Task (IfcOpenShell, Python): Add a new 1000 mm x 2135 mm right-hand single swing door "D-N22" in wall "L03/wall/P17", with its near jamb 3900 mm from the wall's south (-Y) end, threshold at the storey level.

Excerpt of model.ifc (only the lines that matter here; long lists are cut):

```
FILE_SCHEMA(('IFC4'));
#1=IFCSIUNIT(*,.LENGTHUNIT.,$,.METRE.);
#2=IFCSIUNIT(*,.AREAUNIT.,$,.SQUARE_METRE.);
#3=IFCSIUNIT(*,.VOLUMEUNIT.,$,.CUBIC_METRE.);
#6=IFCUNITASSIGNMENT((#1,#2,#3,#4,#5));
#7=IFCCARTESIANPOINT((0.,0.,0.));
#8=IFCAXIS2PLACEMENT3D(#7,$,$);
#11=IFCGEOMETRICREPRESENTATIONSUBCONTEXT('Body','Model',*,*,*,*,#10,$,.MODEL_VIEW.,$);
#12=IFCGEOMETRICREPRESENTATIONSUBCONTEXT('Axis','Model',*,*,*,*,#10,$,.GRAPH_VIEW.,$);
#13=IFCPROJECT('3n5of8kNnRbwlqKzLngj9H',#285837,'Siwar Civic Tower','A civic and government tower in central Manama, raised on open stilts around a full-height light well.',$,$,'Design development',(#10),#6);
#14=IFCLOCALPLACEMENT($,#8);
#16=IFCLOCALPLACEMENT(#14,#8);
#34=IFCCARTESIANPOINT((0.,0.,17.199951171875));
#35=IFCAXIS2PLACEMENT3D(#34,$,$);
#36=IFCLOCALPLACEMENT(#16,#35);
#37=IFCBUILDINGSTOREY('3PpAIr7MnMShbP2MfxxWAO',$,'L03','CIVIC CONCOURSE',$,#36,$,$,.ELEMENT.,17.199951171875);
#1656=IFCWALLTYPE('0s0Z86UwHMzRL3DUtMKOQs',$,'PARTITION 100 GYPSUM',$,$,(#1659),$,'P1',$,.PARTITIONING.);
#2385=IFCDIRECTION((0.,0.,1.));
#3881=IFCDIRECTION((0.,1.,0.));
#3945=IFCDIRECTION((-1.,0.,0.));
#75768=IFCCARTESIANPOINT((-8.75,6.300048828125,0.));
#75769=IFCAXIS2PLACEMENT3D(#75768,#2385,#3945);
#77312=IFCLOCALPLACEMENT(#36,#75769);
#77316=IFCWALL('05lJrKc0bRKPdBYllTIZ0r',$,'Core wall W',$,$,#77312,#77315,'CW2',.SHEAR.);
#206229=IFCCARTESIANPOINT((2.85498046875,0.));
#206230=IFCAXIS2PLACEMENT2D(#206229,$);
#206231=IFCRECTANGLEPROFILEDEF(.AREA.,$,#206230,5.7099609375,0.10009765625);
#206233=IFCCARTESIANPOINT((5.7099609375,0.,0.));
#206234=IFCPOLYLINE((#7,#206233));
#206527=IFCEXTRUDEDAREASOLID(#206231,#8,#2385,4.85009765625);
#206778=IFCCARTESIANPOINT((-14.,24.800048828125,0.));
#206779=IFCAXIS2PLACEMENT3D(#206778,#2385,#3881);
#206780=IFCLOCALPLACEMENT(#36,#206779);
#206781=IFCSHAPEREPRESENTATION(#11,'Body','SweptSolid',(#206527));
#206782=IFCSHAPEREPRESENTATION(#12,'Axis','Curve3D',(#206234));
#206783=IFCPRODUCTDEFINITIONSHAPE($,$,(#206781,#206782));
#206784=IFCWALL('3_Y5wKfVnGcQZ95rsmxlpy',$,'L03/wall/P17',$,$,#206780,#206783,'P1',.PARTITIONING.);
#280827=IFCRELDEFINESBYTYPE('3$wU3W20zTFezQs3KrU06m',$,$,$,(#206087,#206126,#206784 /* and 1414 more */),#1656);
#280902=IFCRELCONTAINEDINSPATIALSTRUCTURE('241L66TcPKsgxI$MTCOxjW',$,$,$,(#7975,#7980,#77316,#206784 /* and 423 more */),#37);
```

```python
import numpy as np
import ifcopenshell
import ifcopenshell.api.feature
import ifcopenshell.api.geometry
import ifcopenshell.api.root
import ifcopenshell.api.spatial
import ifcopenshell.geom
import ifcopenshell.util.element
import ifcopenshell.util.placement
import ifcopenshell.util.representation
import ifcopenshell.util.shape
import ifcopenshell.util.unit

model = ifcopenshell.open("model.ifc")
unit_scale = ifcopenshell.util.unit.calculate_unit_scale(model)
settings = ifcopenshell.geom.settings()


def volume(element):
    """Net volume in cubic metres, openings subtracted."""
    shape = ifcopenshell.geom.create_shape(settings, element)
    return ifcopenshell.util.shape.get_volume(shape.geometry)


wall = model.by_guid("3_Y5wKfVnGcQZ95rsmxlpy")
storey = ifcopenshell.util.element.get_container(wall, ifc_class="IfcBuildingStorey")
context = ifcopenshell.util.representation.get_context(model, "Model", "Body", "MODEL_VIEW")
before = volume(wall)

width, height, from_end, sill = 1, 2.135, 3.9, 0.0  # metres

# The wall runs along its own X axis, and the end named is its -X end.
wall_shape = ifcopenshell.geom.create_shape(settings, wall)
x, y, z = ifcopenshell.util.shape.get_vertices(wall_shape.geometry).T
start = x.min() + from_end
face, thickness = float(y.min()), float(y.max() - y.min())
wall_matrix = ifcopenshell.util.placement.get_local_placement(wall.ObjectPlacement)
level = ifcopenshell.util.placement.get_local_placement(storey.ObjectPlacement)[2, 3]


def in_wall(x, y):
    """Placement at x, y metres in the wall's axes, at sill height."""
    matrix = wall_matrix.copy()
    matrix[:, 3] = wall_matrix @ np.array([x / unit_scale, y / unit_scale, 0.0, 1.0])
    matrix[2, 3] = level + sill / unit_scale
    return matrix


# Opening: a box that overshoots both wall faces by 50 mm.
opening = ifcopenshell.api.root.create_entity(model, ifc_class="IfcOpeningElement", predefined_type="OPENING")
box = ifcopenshell.api.geometry.add_wall_representation(
    model, context=context, length=width, height=height, thickness=thickness + 0.1
)
ifcopenshell.api.geometry.assign_representation(model, product=opening, representation=box)
ifcopenshell.api.geometry.edit_object_placement(model, product=opening, matrix=in_wall(start, face - 0.05), is_si=False)
ifcopenshell.api.feature.add_feature(model, feature=opening, element=wall)

door = ifcopenshell.api.root.create_entity(model, ifc_class="IfcDoor", name="D-N22", predefined_type="DOOR")
door.OverallWidth, door.OverallHeight = width / unit_scale, height / unit_scale
door.OperationType = "SINGLE_SWING_RIGHT"
body = ifcopenshell.api.geometry.add_door_representation(
    model,
    context=context,
    overall_width=door.OverallWidth,
    overall_height=door.OverallHeight,
    operation_type="SINGLE_SWING_RIGHT",
    lining_properties={"LiningDepth": thickness / unit_scale, "ThresholdDepth": thickness / unit_scale},
)
ifcopenshell.api.geometry.assign_representation(model, product=door, representation=body)
ifcopenshell.api.spatial.assign_container(model, products=[door], relating_structure=storey)
ifcopenshell.api.feature.add_filling(model, opening=opening, element=door)

# The lining spans the wall, so the door starts at the wall face.
ifcopenshell.api.geometry.edit_object_placement(model, product=door, matrix=in_wall(start, face), is_si=False)

after = volume(wall)

print(f"wall volume {before:.3f} -> {after:.3f} m3")

model.write("model_v2.ifc")
```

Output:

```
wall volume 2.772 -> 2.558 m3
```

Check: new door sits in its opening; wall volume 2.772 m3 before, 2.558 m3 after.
